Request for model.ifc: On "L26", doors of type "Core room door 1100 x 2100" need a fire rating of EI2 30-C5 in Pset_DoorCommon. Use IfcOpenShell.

First a look at what the model holds.

```python
import ifcopenshell
import ifcopenshell.util.element

model = ifcopenshell.open("model.ifc")
print(model.schema)
storey = next(s for s in model.by_type("IfcBuildingStorey") if s.Name == "L26")
doors = [e for e in ifcopenshell.util.element.get_decomposition(storey) if e.is_a("IfcDoor")]
seen = {}
for e in doors:
    element_type = ifcopenshell.util.element.get_type(e)
    key = (element_type.Name if element_type != e and element_type else None, ifcopenshell.util.element.get_pset(e, "Pset_DoorCommon", "FireRating"))
    seen[key] = seen.get(key, 0) + 1
for (name, value), count in sorted(seen.items(), key=str):
    print(count, "x", name, "|", value)
```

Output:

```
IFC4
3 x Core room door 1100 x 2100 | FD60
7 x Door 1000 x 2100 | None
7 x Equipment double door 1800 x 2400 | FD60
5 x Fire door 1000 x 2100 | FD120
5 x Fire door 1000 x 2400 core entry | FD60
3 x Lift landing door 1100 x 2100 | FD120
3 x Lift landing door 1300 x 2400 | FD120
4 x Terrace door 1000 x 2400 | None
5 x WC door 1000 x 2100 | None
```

```python
import ifcopenshell
import ifcopenshell.api.pset
import ifcopenshell.util.element

model = ifcopenshell.open("model.ifc")

storey = next(s for s in model.by_type("IfcBuildingStorey") if s.Name == "L26")
doors = [e for e in ifcopenshell.util.element.get_decomposition(storey) if e.is_a("IfcDoor")]

count = 0
for e in doors:
    element_type = ifcopenshell.util.element.get_type(e)
    if element_type in (None, e) or element_type.Name != "Core room door 1100 x 2100":
        continue
    # add_pset returns the element's existing set when there is one.
    pset = ifcopenshell.api.pset.add_pset(model, product=e, name="Pset_DoorCommon")
    ifcopenshell.api.pset.edit_pset(model, pset=pset, properties={"FireRating": "EI2 30-C5"})
    count += 1

print(count, "doors updated")

model.write("model_updated.ifc")
```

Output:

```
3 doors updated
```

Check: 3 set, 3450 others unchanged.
